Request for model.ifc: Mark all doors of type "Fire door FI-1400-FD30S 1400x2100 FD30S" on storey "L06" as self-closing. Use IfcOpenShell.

First a look at what the model holds.

```python
import ifcopenshell
import ifcopenshell.util.element

model = ifcopenshell.open("model.ifc")
print(model.schema)
storey = next(s for s in model.by_type("IfcBuildingStorey") if s.Name == "L06")
doors = [e for e in ifcopenshell.util.element.get_decomposition(storey) if e.is_a("IfcDoor")]
seen = {}
for e in doors:
    element_type = ifcopenshell.util.element.get_type(e)
    key = (element_type.Name if element_type != e and element_type else None, ifcopenshell.util.element.get_pset(e, "Pset_DoorCommon", "SelfClosing"))
    seen[key] = seen.get(key, 0) + 1
for (name, value), count in sorted(seen.items(), key=str):
    print(count, "x", name, "|", value)
```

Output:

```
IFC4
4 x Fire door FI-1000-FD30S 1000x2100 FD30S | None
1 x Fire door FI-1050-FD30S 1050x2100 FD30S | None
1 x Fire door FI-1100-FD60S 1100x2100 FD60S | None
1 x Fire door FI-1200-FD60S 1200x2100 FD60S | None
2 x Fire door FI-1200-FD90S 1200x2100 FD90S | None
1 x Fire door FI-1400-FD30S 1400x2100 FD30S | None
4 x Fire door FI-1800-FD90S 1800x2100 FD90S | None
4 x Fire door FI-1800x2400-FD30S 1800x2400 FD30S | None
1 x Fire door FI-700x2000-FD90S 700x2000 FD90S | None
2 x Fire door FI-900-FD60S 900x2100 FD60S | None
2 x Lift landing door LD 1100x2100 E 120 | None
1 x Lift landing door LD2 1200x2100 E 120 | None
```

```python
import ifcopenshell
import ifcopenshell.api.pset
import ifcopenshell.util.element

model = ifcopenshell.open("model.ifc")

storey = next(s for s in model.by_type("IfcBuildingStorey") if s.Name == "L06")
doors = [e for e in ifcopenshell.util.element.get_decomposition(storey) if e.is_a("IfcDoor")]

count = 0
for e in doors:
    element_type = ifcopenshell.util.element.get_type(e)
    if element_type in (None, e) or element_type.Name != "Fire door FI-1400-FD30S 1400x2100 FD30S":
        continue
    # add_pset returns the element's existing set when there is one.
    pset = ifcopenshell.api.pset.add_pset(model, product=e, name="Pset_DoorCommon")
    ifcopenshell.api.pset.edit_pset(model, pset=pset, properties={"SelfClosing": True})
    count += 1

print(count, "doors updated")

model.write("model_updated.ifc")
```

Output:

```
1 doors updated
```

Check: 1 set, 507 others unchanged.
